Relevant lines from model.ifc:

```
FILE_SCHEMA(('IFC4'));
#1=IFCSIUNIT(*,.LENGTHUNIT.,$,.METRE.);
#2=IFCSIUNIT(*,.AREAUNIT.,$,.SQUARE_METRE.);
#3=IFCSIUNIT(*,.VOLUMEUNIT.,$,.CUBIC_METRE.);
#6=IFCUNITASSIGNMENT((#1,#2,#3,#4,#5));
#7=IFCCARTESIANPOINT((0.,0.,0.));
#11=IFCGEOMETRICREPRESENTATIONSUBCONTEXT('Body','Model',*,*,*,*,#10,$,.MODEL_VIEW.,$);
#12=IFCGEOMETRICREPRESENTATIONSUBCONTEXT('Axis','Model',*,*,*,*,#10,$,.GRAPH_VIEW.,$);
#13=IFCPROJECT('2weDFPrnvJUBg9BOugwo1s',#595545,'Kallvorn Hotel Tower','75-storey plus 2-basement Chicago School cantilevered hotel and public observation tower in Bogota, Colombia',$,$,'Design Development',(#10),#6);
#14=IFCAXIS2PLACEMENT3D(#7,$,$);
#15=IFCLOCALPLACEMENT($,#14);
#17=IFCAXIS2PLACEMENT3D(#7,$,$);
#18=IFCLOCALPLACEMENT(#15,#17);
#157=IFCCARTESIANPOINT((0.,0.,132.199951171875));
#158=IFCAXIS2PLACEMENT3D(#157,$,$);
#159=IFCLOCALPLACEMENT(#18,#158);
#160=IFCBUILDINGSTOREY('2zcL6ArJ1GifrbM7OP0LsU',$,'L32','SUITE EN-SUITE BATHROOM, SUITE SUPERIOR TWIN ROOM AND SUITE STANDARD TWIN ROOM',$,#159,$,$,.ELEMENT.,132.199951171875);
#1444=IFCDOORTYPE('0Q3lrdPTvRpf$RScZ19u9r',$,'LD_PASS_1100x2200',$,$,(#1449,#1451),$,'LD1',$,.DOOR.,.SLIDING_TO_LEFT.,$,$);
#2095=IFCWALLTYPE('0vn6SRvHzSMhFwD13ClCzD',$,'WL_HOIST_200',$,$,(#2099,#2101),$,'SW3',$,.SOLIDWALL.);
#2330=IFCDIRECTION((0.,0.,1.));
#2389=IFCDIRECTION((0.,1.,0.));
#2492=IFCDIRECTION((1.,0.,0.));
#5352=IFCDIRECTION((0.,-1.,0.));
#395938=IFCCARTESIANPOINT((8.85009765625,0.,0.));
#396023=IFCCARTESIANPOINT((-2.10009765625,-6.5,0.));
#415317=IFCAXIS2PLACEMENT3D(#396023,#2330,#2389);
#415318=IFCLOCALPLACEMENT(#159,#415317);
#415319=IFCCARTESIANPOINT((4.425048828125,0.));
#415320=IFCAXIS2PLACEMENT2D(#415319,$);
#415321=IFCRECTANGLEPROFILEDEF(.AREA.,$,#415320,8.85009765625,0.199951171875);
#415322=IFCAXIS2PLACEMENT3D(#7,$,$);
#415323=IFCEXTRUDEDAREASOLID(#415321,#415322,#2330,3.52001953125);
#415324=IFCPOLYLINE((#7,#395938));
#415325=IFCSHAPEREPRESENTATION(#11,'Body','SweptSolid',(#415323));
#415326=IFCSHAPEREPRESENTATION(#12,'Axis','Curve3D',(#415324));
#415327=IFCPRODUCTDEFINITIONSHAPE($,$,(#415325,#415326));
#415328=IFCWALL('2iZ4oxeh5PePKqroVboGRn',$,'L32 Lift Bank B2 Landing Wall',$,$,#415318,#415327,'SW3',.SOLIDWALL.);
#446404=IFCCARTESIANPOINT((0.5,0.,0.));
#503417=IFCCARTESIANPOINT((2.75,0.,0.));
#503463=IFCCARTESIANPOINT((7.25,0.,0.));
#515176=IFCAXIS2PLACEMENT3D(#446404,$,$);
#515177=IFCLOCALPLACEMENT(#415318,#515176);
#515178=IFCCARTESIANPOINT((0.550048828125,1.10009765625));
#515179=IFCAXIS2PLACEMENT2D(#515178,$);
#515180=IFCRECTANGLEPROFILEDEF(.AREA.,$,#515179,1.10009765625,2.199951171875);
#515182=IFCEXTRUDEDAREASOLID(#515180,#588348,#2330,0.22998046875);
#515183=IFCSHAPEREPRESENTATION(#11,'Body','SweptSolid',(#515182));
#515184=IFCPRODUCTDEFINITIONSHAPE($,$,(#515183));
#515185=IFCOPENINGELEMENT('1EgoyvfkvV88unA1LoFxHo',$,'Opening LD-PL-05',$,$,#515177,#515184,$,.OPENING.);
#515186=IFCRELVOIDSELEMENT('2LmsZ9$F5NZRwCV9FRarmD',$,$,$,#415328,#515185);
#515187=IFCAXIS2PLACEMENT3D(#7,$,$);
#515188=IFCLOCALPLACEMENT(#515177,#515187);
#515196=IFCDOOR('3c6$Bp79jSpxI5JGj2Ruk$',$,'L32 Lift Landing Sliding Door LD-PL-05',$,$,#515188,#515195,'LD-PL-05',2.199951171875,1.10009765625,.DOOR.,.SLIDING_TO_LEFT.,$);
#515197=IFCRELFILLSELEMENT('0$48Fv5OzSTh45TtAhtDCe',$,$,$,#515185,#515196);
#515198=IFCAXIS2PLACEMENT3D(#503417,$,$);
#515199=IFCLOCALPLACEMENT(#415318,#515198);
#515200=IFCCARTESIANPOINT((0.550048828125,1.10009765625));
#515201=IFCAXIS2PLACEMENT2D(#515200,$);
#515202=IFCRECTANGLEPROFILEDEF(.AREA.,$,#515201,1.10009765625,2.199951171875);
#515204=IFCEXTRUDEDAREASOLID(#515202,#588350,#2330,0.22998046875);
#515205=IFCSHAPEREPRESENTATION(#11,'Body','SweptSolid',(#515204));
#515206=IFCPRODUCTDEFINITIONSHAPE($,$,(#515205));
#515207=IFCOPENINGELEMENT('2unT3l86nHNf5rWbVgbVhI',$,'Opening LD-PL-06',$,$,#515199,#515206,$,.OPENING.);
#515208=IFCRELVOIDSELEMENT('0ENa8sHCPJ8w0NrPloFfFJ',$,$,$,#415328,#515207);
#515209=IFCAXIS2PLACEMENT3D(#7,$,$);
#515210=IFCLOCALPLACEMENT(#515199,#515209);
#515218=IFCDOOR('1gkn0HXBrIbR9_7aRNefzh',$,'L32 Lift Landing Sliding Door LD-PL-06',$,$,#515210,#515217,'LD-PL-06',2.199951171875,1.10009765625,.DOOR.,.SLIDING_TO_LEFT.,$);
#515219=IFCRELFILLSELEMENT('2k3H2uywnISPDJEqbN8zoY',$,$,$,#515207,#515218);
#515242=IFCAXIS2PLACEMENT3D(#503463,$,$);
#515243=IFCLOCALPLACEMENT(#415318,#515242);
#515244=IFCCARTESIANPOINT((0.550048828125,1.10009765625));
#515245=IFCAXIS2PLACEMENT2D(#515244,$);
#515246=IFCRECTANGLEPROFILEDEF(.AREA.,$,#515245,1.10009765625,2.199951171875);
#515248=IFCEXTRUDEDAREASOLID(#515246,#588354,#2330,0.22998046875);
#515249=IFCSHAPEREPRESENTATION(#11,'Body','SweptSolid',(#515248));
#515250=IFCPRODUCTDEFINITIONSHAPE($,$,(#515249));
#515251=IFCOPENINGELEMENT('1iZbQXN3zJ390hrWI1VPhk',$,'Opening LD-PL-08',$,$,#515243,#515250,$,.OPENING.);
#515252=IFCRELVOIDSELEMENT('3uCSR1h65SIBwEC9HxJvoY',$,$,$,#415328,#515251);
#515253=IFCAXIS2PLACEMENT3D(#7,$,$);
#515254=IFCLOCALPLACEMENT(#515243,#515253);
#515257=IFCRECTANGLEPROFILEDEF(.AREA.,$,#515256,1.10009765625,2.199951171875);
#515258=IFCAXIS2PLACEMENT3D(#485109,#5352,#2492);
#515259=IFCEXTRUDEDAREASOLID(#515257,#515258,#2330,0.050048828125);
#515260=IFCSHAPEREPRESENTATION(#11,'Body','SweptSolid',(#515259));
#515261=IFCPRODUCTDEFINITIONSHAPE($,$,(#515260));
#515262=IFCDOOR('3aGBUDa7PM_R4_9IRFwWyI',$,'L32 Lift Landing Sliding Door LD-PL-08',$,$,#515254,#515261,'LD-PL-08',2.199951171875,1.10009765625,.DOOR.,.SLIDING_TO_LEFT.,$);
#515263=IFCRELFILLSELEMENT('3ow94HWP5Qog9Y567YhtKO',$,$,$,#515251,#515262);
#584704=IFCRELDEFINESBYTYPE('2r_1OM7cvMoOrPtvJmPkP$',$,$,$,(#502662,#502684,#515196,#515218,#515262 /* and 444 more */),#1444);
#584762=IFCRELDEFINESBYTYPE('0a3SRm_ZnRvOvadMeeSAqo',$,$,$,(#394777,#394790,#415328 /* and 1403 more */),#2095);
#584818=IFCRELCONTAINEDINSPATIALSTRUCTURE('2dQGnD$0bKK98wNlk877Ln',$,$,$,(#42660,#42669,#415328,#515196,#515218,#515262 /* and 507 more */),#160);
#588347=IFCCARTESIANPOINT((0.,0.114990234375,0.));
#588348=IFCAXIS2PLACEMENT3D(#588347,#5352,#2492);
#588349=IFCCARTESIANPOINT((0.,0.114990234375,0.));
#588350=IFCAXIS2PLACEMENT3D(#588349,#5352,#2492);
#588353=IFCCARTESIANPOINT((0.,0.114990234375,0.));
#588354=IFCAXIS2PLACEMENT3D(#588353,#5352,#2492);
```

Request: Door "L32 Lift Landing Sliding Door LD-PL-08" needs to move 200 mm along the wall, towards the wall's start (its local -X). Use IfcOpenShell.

```python
import ifcopenshell
import ifcopenshell.api.geometry
import ifcopenshell.util.placement
import ifcopenshell.util.unit

model = ifcopenshell.open("model.ifc")
unit_scale = ifcopenshell.util.unit.calculate_unit_scale(model)

door = model.by_guid("3aGBUDa7PM_R4_9IRFwWyI")
opening = door.FillsVoids[0].RelatingOpeningElement
wall = opening.VoidsElements[0].RelatingBuildingElement

wall_matrix = ifcopenshell.util.placement.get_local_placement(wall.ObjectPlacement)
shift = wall_matrix[:3, 0] * -0.2 / unit_scale
before = ifcopenshell.util.placement.get_local_placement(door.ObjectPlacement)[:3, 3].copy()

# The door is placed relative to its opening, so it follows when the opening moves.
matrix = ifcopenshell.util.placement.get_local_placement(opening.ObjectPlacement)
matrix[:3, 3] += shift
ifcopenshell.api.geometry.edit_object_placement(
    model, product=opening, matrix=matrix, is_si=False, should_transform_children=True
)

after = ifcopenshell.util.placement.get_local_placement(door.ObjectPlacement)[:3, 3]
print("door moved by", (after - before).round(3) + 0.0)

model.write("model_updated.ifc")
```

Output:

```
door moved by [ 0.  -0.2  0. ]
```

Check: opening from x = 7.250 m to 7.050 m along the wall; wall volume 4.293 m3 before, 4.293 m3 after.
